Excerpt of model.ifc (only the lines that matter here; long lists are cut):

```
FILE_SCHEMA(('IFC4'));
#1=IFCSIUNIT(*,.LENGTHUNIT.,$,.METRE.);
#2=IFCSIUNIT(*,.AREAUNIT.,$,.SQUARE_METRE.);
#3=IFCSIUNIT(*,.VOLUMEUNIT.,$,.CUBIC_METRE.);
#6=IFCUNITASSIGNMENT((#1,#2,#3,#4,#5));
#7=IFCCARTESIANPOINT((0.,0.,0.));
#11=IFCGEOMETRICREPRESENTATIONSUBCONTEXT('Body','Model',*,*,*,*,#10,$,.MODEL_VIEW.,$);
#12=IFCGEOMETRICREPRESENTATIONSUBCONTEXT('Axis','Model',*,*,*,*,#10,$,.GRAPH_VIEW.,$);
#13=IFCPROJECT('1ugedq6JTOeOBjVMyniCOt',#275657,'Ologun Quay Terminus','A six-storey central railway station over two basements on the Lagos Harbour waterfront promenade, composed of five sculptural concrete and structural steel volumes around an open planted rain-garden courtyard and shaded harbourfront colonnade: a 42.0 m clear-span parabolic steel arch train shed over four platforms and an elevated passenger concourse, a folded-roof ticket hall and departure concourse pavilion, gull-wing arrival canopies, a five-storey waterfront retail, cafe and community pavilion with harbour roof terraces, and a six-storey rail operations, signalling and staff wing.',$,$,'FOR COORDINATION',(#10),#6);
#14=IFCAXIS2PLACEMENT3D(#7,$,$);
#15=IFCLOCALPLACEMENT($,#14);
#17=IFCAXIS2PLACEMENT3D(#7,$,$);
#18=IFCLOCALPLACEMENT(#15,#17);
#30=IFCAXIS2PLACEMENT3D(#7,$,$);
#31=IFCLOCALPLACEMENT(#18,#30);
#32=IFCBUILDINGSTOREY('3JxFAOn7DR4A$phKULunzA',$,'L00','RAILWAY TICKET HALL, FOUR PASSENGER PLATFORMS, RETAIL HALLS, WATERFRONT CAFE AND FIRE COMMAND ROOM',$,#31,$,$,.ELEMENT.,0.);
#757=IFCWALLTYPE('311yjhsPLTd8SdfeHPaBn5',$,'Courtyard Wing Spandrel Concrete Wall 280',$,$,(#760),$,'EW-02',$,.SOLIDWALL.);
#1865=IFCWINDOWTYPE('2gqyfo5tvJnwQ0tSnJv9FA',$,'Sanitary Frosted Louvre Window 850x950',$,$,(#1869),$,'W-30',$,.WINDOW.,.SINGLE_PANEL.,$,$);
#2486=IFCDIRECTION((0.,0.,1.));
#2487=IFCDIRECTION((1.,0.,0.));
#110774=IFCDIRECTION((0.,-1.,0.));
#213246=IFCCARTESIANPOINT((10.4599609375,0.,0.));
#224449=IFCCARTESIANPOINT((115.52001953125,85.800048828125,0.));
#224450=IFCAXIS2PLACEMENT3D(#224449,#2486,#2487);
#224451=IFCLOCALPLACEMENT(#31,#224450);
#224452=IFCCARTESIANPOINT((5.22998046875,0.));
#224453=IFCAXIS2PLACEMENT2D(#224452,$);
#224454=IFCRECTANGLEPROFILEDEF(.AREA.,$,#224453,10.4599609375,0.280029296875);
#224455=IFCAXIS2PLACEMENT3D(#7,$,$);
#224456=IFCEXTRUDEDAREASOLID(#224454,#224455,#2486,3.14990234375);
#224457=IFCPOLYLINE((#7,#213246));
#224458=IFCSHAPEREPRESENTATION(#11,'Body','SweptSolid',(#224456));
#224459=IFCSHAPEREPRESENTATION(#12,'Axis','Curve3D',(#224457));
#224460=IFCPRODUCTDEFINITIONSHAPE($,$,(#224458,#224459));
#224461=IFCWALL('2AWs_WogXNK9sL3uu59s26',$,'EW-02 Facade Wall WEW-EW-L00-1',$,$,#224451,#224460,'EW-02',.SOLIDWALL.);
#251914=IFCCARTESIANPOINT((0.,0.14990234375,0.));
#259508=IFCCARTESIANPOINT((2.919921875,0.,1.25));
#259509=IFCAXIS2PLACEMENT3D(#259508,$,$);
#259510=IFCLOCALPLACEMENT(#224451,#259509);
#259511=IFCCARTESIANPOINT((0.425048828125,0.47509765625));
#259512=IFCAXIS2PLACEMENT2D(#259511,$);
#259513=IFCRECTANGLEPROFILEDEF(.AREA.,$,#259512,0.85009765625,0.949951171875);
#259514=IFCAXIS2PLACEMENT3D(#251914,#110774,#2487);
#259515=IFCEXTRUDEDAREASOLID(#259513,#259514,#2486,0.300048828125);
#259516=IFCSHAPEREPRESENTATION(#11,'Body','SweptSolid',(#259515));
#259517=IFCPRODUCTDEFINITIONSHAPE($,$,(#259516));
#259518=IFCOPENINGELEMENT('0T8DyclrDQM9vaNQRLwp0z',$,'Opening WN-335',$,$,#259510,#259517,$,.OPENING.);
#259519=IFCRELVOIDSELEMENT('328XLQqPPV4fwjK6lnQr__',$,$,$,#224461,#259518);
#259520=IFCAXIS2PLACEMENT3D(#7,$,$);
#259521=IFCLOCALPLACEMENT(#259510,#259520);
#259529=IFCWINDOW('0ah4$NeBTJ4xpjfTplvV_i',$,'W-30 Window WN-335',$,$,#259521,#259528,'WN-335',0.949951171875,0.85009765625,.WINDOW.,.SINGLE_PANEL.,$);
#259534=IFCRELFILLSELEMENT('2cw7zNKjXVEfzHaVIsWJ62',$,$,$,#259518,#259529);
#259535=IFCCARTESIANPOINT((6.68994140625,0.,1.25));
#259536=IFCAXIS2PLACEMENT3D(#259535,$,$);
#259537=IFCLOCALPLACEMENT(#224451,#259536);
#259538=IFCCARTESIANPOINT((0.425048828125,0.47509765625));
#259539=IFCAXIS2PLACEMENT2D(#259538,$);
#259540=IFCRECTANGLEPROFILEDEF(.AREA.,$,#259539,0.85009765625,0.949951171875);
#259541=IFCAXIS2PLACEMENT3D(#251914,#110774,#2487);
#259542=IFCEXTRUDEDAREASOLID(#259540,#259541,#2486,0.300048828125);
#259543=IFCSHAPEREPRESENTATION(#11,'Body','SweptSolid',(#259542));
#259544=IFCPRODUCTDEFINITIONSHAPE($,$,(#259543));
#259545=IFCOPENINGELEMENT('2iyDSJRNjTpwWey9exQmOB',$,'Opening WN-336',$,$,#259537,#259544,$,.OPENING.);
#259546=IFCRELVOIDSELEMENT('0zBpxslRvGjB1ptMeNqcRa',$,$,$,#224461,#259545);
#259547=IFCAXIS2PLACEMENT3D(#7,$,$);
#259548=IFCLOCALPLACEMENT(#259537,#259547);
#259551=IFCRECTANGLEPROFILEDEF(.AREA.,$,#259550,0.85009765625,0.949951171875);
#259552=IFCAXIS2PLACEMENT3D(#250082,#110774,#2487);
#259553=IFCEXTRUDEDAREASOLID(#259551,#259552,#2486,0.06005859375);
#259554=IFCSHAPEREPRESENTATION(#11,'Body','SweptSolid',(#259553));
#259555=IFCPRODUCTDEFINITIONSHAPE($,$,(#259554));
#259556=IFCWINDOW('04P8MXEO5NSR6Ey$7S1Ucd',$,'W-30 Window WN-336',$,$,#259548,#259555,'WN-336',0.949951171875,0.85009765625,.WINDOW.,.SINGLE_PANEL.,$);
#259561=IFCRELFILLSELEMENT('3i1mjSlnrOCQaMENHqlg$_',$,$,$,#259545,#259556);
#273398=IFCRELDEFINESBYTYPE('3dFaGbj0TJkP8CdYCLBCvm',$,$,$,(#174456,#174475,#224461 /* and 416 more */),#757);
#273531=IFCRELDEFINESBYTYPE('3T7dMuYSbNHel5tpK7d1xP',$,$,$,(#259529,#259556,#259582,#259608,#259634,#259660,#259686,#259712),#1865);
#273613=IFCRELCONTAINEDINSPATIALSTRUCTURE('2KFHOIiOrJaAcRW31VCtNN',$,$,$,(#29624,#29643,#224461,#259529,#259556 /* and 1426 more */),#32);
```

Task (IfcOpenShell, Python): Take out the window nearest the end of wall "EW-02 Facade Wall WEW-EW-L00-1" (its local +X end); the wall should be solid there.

```python
import ifcopenshell
import ifcopenshell.api.feature
import ifcopenshell.api.root
import ifcopenshell.geom
import ifcopenshell.util.shape

model = ifcopenshell.open("model.ifc")
settings = ifcopenshell.geom.settings()


def volume(element):
    """Net volume in cubic metres, openings subtracted."""
    shape = ifcopenshell.geom.create_shape(settings, element)
    return ifcopenshell.util.shape.get_volume(shape.geometry)


window = model.by_id(259556)
opening = window.FillsVoids[0].RelatingOpeningElement
wall = opening.VoidsElements[0].RelatingBuildingElement
before = volume(wall)

ifcopenshell.api.root.remove_product(model, product=window)
ifcopenshell.api.feature.remove_feature(model, feature=opening)

after = volume(wall)

print(f"wall volume {before:.3f} -> {after:.3f} m3")

model.write("model_updated.ifc")
```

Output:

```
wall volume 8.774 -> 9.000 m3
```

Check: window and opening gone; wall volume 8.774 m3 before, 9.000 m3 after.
